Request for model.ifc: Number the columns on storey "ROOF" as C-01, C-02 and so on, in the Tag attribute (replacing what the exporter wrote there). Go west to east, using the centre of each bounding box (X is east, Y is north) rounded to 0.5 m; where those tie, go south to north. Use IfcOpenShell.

First a look at what the model holds.

```python
import ifcopenshell
import ifcopenshell.util.element
import ifcopenshell.util.placement

model = ifcopenshell.open("model.ifc")
print(model.schema)
storey = next(s for s in model.by_type("IfcBuildingStorey") if s.Name == "ROOF")
columns = [e for e in ifcopenshell.util.element.get_decomposition(storey) if e.is_a("IfcColumn")]
for e in sorted(columns, key=lambda e: e.id()):
    origin = ifcopenshell.util.placement.get_local_placement(e.ObjectPlacement)[:3, 3]
    print(e.id(), e.Tag, e.Name, origin.round(2) + 0.0, sep=" | ")
```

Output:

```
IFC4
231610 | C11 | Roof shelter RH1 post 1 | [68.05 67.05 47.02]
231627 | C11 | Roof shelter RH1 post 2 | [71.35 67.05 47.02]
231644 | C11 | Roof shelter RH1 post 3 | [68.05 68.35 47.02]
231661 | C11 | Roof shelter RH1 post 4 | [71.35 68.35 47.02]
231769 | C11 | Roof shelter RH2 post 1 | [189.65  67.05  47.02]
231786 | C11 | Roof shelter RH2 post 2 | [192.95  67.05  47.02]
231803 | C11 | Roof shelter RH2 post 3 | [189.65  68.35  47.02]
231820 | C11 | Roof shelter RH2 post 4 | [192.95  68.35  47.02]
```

```python
import ifcopenshell
import ifcopenshell.geom
import ifcopenshell.util.element
import ifcopenshell.util.shape

model = ifcopenshell.open("model.ifc")
settings = ifcopenshell.geom.settings()
settings.set("use-world-coords", True)


def centre(element):
    shape = ifcopenshell.geom.create_shape(settings, element)
    return ifcopenshell.util.shape.get_bbox_centroid(shape.geometry)


storey = next(s for s in model.by_type("IfcBuildingStorey") if s.Name == "ROOF")
columns = [e for e in ifcopenshell.util.element.get_decomposition(storey) if e.is_a("IfcColumn")]

# Insertion points can sit at a corner or the storey origin, so sort by the geometry (in metres).
centres = {e: centre(e) for e in columns}
columns.sort(key=lambda e: (round(centres[e][0] / 0.5), centres[e][1]))

for i, e in enumerate(columns, start=1):
    number = f"C-{i:02d}"
    e.Tag = number
    print(e.id(), number)

model.write("model_v2.ifc")
```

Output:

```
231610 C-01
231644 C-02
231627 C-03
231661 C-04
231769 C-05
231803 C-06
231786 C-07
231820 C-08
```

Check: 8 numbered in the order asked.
